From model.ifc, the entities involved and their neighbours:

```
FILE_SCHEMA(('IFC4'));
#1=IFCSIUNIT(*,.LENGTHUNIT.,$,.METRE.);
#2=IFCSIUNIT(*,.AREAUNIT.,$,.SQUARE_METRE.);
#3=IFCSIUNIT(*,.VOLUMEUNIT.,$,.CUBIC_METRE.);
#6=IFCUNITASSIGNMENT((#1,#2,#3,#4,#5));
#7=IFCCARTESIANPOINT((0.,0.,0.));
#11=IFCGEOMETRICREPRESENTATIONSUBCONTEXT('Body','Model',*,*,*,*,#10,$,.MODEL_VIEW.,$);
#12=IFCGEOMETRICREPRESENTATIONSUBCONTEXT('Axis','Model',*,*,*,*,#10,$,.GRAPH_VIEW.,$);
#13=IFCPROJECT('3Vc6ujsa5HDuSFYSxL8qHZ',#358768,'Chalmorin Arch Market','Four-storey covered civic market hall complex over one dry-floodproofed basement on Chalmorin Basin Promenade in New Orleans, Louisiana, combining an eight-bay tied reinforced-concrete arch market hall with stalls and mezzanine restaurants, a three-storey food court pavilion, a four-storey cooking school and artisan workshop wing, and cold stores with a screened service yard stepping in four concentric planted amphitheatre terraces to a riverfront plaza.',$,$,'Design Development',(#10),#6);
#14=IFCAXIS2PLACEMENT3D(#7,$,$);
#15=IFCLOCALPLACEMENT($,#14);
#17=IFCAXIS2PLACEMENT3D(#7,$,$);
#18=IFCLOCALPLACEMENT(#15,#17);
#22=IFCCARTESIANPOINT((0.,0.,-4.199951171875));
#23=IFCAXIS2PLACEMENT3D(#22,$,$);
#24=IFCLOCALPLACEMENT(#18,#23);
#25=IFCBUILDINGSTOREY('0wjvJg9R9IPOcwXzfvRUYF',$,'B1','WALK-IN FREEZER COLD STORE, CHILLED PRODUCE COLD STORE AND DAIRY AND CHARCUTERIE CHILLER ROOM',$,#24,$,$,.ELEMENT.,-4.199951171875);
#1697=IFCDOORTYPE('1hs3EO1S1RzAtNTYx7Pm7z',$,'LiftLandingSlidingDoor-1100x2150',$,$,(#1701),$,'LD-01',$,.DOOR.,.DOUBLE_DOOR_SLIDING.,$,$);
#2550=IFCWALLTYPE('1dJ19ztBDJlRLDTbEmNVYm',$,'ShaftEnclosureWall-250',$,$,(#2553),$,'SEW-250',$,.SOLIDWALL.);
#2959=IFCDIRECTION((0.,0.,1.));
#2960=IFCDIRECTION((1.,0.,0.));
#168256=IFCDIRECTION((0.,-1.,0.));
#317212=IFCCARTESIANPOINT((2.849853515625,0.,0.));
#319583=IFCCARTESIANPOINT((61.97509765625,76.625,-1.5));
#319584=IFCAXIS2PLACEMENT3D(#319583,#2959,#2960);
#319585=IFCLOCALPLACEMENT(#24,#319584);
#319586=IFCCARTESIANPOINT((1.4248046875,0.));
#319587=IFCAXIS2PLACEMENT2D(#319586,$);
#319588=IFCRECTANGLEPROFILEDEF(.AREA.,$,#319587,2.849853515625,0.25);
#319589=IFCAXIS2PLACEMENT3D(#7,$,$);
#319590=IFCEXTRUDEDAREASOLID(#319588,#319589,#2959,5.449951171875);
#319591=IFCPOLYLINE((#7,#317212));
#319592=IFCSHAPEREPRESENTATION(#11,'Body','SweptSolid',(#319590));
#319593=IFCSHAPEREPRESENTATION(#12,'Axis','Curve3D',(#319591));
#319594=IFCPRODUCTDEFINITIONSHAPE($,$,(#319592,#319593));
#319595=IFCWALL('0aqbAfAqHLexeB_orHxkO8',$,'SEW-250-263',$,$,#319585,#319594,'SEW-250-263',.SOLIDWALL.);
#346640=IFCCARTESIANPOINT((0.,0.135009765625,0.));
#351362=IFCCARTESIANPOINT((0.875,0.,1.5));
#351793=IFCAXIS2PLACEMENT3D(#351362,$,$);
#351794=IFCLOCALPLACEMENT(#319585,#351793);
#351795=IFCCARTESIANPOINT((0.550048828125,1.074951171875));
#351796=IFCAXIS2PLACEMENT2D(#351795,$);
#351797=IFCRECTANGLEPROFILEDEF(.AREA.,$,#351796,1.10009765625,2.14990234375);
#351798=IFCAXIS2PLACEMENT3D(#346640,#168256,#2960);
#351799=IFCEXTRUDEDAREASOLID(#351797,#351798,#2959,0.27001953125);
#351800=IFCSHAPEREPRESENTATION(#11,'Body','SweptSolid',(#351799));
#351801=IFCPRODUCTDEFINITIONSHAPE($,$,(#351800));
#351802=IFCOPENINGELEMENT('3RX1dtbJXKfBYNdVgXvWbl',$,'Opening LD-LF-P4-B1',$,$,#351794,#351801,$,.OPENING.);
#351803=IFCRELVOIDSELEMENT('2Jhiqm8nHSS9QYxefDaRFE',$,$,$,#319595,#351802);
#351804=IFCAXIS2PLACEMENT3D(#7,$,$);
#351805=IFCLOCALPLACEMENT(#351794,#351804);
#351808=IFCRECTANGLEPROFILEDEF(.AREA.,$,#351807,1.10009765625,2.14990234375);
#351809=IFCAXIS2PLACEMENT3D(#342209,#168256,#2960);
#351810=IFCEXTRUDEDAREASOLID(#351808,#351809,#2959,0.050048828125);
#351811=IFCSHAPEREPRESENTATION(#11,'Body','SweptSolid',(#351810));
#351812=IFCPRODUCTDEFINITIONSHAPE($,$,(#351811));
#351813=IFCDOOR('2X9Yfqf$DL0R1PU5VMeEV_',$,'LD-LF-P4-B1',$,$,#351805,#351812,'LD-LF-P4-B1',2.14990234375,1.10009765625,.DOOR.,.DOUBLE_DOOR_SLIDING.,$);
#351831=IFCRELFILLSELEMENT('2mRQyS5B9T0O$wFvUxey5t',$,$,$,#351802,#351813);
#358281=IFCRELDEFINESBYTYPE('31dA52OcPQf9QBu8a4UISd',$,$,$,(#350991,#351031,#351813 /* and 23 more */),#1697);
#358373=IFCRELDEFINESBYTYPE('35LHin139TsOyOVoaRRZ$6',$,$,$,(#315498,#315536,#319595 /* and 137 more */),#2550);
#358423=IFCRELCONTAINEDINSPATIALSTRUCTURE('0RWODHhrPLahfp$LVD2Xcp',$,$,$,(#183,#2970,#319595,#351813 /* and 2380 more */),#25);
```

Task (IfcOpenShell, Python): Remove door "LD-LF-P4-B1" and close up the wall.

```python
import ifcopenshell
import ifcopenshell.api.feature
import ifcopenshell.api.root
import ifcopenshell.geom
import ifcopenshell.util.shape

model = ifcopenshell.open("model.ifc")
settings = ifcopenshell.geom.settings()


def volume(element):
    """Net volume in cubic metres, openings subtracted."""
    shape = ifcopenshell.geom.create_shape(settings, element)
    return ifcopenshell.util.shape.get_volume(shape.geometry)


door = model.by_guid("2X9Yfqf$DL0R1PU5VMeEV_")
opening = door.FillsVoids[0].RelatingOpeningElement
wall = opening.VoidsElements[0].RelatingBuildingElement
before = volume(wall)

ifcopenshell.api.root.remove_product(model, product=door)
ifcopenshell.api.feature.remove_feature(model, feature=opening)

after = volume(wall)

print(f"wall volume {before:.3f} -> {after:.3f} m3")

model.write("model-out.ifc")
```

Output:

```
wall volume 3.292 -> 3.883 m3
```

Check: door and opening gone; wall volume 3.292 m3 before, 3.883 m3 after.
